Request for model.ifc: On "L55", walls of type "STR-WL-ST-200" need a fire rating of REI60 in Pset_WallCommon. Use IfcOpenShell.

First a look at what the model holds.

```python
import ifcopenshell
import ifcopenshell.util.element

model = ifcopenshell.open("model.ifc")
print(model.schema)
storey = next(s for s in model.by_type("IfcBuildingStorey") if s.Name == "L55")
walls = [e for e in ifcopenshell.util.element.get_decomposition(storey) if e.is_a("IfcWall")]
seen = {}
for e in walls:
    element_type = ifcopenshell.util.element.get_type(e)
    key = (element_type.Name if element_type != e and element_type else None, ifcopenshell.util.element.get_pset(e, "Pset_WallCommon", "FireRating"))
    seen[key] = seen.get(key, 0) + 1
for (name, value), count in sorted(seen.items(), key=str):
    print(count, "x", name, "|", value)
```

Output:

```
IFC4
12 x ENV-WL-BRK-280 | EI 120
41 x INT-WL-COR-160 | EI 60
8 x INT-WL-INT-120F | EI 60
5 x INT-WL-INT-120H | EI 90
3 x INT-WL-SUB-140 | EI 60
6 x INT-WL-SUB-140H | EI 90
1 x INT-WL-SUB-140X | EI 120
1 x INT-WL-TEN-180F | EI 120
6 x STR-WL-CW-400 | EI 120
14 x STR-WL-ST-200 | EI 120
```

```python
import ifcopenshell
import ifcopenshell.api.pset
import ifcopenshell.util.element

model = ifcopenshell.open("model.ifc")

storey = next(s for s in model.by_type("IfcBuildingStorey") if s.Name == "L55")
walls = [e for e in ifcopenshell.util.element.get_decomposition(storey) if e.is_a("IfcWall")]

count = 0
for e in walls:
    element_type = ifcopenshell.util.element.get_type(e)
    if element_type in (None, e) or element_type.Name != "STR-WL-ST-200":
        continue
    # add_pset returns the element's existing set when there is one.
    pset = ifcopenshell.api.pset.add_pset(model, product=e, name="Pset_WallCommon")
    ifcopenshell.api.pset.edit_pset(model, pset=pset, properties={"FireRating": "REI60"})
    count += 1

print(count, "walls updated")

model.write("model-out.ifc")
```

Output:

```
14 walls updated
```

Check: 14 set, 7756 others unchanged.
